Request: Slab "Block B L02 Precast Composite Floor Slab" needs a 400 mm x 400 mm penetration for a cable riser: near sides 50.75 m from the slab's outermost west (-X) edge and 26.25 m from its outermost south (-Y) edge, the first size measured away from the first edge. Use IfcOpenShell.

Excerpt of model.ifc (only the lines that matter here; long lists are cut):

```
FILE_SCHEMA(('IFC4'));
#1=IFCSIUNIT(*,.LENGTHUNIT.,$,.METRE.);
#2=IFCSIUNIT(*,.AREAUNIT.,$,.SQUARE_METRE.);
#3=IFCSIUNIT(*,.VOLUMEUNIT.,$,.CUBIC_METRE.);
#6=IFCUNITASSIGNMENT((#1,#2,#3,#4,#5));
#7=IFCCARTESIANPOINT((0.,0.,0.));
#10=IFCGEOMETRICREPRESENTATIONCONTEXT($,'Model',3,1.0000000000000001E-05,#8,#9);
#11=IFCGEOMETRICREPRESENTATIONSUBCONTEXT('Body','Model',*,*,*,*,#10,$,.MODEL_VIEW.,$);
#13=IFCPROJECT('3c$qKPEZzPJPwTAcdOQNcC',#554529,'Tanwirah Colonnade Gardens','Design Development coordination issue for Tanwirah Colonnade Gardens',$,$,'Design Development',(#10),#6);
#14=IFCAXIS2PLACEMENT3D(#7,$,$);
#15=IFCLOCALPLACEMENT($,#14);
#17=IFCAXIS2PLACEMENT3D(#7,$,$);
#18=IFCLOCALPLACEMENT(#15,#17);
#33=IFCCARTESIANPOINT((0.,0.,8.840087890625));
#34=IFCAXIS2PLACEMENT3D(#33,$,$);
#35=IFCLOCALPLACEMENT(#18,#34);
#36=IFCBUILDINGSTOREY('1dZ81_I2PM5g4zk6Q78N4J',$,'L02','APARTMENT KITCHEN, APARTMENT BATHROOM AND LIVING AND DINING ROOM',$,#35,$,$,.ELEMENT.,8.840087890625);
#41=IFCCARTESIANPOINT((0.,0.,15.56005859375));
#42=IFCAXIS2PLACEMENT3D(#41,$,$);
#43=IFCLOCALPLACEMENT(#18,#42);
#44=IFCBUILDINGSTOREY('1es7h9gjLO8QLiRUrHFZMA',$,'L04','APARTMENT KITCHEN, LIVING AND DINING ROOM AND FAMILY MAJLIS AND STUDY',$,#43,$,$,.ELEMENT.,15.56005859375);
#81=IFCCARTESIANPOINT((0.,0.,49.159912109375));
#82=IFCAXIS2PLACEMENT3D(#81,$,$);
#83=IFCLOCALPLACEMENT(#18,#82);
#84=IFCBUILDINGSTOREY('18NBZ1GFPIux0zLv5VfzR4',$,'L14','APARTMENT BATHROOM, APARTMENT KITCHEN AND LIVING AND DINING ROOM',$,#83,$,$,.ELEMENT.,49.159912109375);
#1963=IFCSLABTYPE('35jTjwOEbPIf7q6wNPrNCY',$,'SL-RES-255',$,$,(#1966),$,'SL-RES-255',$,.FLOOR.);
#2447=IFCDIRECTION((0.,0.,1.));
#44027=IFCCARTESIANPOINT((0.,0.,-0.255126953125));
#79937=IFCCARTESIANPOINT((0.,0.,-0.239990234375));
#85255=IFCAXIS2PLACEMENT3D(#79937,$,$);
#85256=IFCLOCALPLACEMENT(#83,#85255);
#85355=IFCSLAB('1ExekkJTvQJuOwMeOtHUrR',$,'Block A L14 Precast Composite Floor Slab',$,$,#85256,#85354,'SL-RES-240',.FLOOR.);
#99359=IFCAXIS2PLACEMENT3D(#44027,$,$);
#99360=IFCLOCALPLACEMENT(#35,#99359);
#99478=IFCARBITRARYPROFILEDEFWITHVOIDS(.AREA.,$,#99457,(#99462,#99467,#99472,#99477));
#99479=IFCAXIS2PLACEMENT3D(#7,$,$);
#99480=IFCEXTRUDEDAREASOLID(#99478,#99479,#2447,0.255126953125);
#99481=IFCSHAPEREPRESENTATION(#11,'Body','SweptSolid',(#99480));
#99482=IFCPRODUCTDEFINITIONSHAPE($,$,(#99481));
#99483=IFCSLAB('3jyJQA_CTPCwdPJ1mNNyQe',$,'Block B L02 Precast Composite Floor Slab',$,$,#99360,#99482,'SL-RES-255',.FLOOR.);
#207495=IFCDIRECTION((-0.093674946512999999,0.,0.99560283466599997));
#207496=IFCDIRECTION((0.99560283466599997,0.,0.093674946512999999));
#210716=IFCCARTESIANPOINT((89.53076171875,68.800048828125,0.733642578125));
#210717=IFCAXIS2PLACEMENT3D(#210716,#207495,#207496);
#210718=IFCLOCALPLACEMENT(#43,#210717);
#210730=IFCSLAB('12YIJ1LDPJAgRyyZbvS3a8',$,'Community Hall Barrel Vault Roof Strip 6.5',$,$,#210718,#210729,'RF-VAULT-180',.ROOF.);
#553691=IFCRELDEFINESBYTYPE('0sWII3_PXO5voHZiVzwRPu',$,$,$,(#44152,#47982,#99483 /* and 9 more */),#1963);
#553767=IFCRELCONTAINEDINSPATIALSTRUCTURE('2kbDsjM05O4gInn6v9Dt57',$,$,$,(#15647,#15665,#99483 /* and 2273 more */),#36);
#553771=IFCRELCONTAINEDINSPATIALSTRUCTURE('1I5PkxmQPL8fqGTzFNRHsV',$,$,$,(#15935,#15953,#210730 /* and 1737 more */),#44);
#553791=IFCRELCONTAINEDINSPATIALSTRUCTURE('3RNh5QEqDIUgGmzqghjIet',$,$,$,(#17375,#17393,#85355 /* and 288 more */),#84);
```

```python
import numpy as np
import ifcopenshell
import ifcopenshell.api.feature
import ifcopenshell.api.geometry
import ifcopenshell.api.root
import ifcopenshell.geom
import ifcopenshell.util.placement
import ifcopenshell.util.representation
import ifcopenshell.util.shape
import ifcopenshell.util.unit

model = ifcopenshell.open("model.ifc")
unit_scale = ifcopenshell.util.unit.calculate_unit_scale(model)
settings = ifcopenshell.geom.settings()


def volume(element):
    """Net volume in cubic metres, openings subtracted."""
    shape = ifcopenshell.geom.create_shape(settings, element)
    return ifcopenshell.util.shape.get_volume(shape.geometry)


slab = model.by_guid("3jyJQA_CTPCwdPJ1mNNyQe")
before = volume(slab)

# Extent in the slab's own axes, in metres. The edges named are its -X and -Y sides.
slab_shape = ifcopenshell.geom.create_shape(settings, slab)
vertices = ifcopenshell.util.shape.get_vertices(slab_shape.geometry)
x_min, y_min, bottom = vertices.min(axis=0)
top = vertices[:, 2].max()

opening = ifcopenshell.api.root.create_entity(model, ifc_class="IfcOpeningElement", name="Cable riser opening", predefined_type="OPENING")
context = ifcopenshell.util.representation.get_context(model, "Model", "Body", "MODEL_VIEW")
width, depth = 0.4, 0.4
outline = [(0.0, 0.0), (width, 0.0), (width, depth), (0.0, depth), (0.0, 0.0)]
# Overshoot both faces by 50 mm so the cut is clean.
shape = ifcopenshell.api.geometry.add_slab_representation(
    model, context=context, depth=top - bottom + 0.1, polyline=outline
)
ifcopenshell.api.geometry.assign_representation(model, product=opening, representation=shape)

matrix = ifcopenshell.util.placement.get_local_placement(slab.ObjectPlacement)
matrix[:, 3] = matrix @ np.append(np.array([x_min + 50.75, y_min + 26.25, bottom - 0.05]) / unit_scale, 1.0)
ifcopenshell.api.geometry.edit_object_placement(model, product=opening, matrix=matrix, is_si=False)
ifcopenshell.api.feature.add_feature(model, feature=opening, element=slab)

after = volume(slab)

print(f"slab volume {before:.3f} -> {after:.3f} m3")

model.write("model_edited.ifc")
```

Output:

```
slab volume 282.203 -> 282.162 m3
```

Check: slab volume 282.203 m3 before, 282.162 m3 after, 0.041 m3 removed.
